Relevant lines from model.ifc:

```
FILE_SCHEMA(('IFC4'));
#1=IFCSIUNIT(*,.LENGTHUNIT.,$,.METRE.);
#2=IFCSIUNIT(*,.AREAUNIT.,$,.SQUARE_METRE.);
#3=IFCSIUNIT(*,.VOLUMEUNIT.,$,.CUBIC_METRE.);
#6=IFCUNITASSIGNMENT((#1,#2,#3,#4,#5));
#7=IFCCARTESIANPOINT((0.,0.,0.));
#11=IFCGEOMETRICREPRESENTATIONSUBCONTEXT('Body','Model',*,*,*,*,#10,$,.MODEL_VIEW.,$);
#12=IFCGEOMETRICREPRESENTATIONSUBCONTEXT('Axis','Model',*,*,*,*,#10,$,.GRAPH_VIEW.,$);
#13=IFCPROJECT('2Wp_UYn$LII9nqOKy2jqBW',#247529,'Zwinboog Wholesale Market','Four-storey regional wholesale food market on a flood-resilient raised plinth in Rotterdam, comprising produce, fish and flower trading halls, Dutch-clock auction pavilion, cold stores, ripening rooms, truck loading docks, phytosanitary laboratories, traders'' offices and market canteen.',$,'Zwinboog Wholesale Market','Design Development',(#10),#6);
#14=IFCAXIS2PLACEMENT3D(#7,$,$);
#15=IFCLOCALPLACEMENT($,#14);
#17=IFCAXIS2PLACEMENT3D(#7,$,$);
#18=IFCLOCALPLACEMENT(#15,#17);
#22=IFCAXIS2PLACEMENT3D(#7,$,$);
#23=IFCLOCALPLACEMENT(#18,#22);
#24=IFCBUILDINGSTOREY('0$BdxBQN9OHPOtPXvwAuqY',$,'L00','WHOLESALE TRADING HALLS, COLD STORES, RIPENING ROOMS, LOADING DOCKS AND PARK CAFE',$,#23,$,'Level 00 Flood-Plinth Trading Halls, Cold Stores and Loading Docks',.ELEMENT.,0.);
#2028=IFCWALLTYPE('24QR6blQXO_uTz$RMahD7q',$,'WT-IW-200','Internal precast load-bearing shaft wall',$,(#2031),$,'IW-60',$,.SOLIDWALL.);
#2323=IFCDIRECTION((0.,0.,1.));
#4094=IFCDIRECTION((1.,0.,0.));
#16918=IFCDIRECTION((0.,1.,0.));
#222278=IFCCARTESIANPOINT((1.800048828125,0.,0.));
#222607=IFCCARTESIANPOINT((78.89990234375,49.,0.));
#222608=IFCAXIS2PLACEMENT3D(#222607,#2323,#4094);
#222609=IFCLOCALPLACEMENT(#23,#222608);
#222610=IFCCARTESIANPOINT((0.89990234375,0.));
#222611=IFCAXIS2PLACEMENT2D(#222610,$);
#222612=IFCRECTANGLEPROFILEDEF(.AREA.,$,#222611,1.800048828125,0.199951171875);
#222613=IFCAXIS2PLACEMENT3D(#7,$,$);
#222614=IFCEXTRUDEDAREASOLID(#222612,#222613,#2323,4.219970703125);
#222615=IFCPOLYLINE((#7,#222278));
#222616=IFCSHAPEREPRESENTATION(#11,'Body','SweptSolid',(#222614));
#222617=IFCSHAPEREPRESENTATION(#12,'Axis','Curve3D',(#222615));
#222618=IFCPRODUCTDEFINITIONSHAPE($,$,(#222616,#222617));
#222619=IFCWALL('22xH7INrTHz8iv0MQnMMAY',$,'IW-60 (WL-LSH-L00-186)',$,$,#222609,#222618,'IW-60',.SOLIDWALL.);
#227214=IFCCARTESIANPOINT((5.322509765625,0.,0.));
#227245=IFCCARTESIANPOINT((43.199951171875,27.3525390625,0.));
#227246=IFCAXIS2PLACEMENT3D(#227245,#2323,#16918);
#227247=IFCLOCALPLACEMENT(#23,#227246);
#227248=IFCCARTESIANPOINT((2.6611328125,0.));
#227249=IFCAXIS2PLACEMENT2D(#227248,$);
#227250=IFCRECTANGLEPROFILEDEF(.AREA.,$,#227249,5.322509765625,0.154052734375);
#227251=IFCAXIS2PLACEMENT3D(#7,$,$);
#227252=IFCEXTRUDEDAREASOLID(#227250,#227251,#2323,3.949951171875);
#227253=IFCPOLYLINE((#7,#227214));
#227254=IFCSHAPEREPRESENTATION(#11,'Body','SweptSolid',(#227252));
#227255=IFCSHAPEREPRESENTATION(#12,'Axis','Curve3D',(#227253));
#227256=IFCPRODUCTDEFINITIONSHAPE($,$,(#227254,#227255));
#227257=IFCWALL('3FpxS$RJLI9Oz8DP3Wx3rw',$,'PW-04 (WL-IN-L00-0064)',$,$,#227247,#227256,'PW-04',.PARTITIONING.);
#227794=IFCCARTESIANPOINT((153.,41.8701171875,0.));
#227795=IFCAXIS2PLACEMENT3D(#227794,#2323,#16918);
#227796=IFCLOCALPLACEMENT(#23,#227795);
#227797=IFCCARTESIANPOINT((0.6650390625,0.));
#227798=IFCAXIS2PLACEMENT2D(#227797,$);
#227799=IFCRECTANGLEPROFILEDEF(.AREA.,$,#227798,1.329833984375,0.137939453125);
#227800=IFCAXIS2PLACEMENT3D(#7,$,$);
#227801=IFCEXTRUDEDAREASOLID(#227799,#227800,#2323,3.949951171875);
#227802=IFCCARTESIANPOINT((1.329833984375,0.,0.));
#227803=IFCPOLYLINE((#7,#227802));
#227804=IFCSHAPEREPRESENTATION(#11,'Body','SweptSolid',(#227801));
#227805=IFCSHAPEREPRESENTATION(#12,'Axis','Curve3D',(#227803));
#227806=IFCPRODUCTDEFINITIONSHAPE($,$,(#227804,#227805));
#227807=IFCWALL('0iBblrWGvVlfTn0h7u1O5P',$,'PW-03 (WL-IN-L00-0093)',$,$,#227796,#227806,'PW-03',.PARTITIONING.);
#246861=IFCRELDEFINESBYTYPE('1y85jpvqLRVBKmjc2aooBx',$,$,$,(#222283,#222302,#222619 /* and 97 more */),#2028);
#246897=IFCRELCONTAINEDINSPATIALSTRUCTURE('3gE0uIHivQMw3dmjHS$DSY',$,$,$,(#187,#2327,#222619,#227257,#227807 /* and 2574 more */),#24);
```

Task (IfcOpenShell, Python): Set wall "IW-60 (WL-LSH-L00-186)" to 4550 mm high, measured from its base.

```python
import ifcopenshell
import ifcopenshell.geom
import ifcopenshell.util.representation
import ifcopenshell.util.shape
import ifcopenshell.util.unit

model = ifcopenshell.open("model.ifc")
unit_scale = ifcopenshell.util.unit.calculate_unit_scale(model)
settings = ifcopenshell.geom.settings()


def volume(element):
    """Net volume in cubic metres, openings subtracted."""
    shape = ifcopenshell.geom.create_shape(settings, element)
    return ifcopenshell.util.shape.get_volume(shape.geometry)


wall = model.by_guid("22xH7INrTHz8iv0MQnMMAY")
before = volume(wall)

body = ifcopenshell.util.representation.get_representation(wall, "Model", "Body")
solid = body.Items[0]
old_height = solid.Depth
solid.Depth = 4.55 / unit_scale
after = volume(wall)

print(f"height {old_height:g} -> {solid.Depth:g}, volume {before:.3f} -> {after:.3f} m3")

model.write("model_edited.ifc")
```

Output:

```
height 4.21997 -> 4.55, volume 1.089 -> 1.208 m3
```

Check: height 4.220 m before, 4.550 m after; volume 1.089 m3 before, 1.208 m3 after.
